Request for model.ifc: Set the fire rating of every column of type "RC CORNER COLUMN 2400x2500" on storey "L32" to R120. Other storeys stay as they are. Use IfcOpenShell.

First a look at what the model holds.

```python
import ifcopenshell
import ifcopenshell.util.element

model = ifcopenshell.open("model.ifc")
print(model.schema)
storey = next(s for s in model.by_type("IfcBuildingStorey") if s.Name == "L32")
columns = [e for e in ifcopenshell.util.element.get_decomposition(storey) if e.is_a("IfcColumn")]
seen = {}
for e in columns:
    element_type = ifcopenshell.util.element.get_type(e)
    key = (element_type.Name if element_type != e and element_type else None, ifcopenshell.util.element.get_pset(e, "Pset_ColumnCommon", "FireRating"))
    seen[key] = seen.get(key, 0) + 1
for (name, value), count in sorted(seen.items(), key=str):
    print(count, "x", name, "|", value)
```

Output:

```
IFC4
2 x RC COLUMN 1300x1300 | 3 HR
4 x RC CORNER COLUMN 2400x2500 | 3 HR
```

```python
import ifcopenshell
import ifcopenshell.api.pset
import ifcopenshell.util.element

model = ifcopenshell.open("model.ifc")

storey = next(s for s in model.by_type("IfcBuildingStorey") if s.Name == "L32")
columns = [e for e in ifcopenshell.util.element.get_decomposition(storey) if e.is_a("IfcColumn")]

count = 0
for e in columns:
    element_type = ifcopenshell.util.element.get_type(e)
    if element_type in (None, e) or element_type.Name != "RC CORNER COLUMN 2400x2500":
        continue
    found = ifcopenshell.util.element.get_pset(e, "Pset_ColumnCommon", should_inherit=False)
    if found:
        pset = model.by_id(found["id"])
        if len(ifcopenshell.util.element.get_elements_by_pset(pset)) > 1:
            pset = ifcopenshell.api.pset.unshare_pset(model, products=[e], pset=pset)[0]
    else:
        pset = ifcopenshell.api.pset.add_pset(model, product=e, name="Pset_ColumnCommon")
    ifcopenshell.api.pset.edit_pset(model, pset=pset, properties={"FireRating": "R120"})
    count += 1

print(count, "columns updated")

model.write("model_rev.ifc")
```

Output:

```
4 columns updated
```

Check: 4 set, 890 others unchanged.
